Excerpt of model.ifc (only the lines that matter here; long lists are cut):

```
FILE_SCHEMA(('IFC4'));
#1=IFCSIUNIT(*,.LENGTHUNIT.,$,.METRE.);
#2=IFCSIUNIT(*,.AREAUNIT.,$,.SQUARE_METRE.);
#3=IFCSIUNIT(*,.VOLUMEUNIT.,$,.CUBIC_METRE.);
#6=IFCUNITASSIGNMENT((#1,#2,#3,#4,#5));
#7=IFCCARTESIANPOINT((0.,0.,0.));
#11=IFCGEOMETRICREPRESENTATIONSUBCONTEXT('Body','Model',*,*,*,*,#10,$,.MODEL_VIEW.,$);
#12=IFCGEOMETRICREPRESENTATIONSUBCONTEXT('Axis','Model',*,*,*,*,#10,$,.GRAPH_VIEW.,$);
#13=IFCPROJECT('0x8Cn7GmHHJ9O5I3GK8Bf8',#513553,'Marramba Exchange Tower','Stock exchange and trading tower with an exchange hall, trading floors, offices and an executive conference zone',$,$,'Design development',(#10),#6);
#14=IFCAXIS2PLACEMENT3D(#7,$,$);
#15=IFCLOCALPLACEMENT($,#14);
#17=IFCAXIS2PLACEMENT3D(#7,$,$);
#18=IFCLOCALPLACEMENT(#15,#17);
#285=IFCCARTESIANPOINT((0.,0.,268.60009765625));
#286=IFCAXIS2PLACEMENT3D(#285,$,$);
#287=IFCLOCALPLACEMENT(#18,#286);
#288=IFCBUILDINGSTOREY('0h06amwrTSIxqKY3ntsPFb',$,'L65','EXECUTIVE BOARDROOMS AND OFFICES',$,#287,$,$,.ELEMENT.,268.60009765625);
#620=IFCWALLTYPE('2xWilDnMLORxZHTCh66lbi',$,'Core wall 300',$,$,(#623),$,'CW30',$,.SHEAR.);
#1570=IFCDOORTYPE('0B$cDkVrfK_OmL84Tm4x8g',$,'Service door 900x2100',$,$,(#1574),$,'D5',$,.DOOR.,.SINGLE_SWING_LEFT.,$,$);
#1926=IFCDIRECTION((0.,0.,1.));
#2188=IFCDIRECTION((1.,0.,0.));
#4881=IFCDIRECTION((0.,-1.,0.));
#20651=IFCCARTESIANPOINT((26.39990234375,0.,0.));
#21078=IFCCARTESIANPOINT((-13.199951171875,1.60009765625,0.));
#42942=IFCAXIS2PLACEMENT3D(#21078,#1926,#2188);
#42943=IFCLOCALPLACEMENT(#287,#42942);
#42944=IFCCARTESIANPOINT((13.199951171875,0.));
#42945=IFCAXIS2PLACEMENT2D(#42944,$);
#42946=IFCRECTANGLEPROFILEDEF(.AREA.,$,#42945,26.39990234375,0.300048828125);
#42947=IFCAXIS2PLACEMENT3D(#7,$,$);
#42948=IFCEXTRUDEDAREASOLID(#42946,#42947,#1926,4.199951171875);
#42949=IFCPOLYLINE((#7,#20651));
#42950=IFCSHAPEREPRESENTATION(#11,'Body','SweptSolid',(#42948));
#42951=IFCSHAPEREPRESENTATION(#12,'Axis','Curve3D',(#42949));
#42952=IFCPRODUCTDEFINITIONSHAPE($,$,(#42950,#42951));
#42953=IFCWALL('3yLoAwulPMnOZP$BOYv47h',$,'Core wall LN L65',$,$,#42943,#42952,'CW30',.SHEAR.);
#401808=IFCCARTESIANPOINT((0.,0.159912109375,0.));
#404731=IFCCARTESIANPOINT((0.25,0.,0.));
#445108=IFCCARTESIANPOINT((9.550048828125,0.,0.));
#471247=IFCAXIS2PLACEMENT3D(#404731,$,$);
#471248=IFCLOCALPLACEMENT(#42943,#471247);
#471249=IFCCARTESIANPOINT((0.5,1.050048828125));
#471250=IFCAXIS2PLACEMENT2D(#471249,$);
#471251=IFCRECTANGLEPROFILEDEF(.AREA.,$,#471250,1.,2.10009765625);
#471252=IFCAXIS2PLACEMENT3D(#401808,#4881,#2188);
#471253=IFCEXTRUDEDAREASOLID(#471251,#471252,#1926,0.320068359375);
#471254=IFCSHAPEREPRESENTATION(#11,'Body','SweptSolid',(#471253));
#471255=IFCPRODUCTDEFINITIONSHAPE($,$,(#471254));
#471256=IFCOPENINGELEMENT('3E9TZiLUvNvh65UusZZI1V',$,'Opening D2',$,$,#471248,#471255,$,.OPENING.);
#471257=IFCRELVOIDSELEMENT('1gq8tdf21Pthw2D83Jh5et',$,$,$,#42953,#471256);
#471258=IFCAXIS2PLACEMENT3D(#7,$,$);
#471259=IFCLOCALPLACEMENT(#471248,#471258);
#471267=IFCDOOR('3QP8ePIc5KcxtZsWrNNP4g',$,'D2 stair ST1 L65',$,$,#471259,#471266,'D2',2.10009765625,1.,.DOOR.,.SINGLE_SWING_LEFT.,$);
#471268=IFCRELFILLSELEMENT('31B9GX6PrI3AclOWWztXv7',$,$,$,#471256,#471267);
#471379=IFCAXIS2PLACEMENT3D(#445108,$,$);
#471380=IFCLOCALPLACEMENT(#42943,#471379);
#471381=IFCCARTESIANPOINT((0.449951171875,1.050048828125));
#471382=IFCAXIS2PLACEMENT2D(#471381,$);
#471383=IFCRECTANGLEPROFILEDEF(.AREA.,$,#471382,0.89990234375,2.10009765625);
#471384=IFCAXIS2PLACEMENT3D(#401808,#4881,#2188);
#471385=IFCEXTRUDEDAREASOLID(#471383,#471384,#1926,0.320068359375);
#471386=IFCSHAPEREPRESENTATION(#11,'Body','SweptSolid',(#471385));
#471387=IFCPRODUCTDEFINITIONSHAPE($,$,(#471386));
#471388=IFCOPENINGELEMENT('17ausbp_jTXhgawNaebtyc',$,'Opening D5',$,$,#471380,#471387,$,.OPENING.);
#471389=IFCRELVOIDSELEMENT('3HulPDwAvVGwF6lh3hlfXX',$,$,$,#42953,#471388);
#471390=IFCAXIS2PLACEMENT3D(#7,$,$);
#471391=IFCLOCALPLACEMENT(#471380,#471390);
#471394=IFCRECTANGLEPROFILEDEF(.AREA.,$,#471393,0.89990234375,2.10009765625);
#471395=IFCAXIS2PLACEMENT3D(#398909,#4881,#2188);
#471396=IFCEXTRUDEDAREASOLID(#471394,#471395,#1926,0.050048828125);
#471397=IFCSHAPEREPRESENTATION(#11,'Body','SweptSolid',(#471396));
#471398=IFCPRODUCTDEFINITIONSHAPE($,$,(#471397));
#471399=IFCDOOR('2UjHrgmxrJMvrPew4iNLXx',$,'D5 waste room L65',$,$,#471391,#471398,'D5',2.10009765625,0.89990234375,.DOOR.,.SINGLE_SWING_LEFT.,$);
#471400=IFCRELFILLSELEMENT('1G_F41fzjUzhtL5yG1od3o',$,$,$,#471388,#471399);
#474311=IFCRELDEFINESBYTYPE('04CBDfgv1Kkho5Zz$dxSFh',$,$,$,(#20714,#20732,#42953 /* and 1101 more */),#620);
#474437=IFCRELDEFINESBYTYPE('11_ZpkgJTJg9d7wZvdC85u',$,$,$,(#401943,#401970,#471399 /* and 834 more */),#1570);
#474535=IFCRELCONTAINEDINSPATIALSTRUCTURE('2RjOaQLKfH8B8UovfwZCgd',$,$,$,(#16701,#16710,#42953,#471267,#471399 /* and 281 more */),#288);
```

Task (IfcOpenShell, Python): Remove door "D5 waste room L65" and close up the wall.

```python
import ifcopenshell
import ifcopenshell.api.feature
import ifcopenshell.api.root
import ifcopenshell.geom
import ifcopenshell.util.shape

model = ifcopenshell.open("model.ifc")
settings = ifcopenshell.geom.settings()


def volume(element):
    """Net volume in cubic metres, openings subtracted."""
    shape = ifcopenshell.geom.create_shape(settings, element)
    return ifcopenshell.util.shape.get_volume(shape.geometry)


door = model.by_id(471399)
opening = door.FillsVoids[0].RelatingOpeningElement
wall = opening.VoidsElements[0].RelatingBuildingElement
before = volume(wall)

ifcopenshell.api.root.remove_product(model, product=door)
ifcopenshell.api.feature.remove_feature(model, feature=opening)

after = volume(wall)

print(f"wall volume {before:.3f} -> {after:.3f} m3")

model.write("model_edited.ifc")
```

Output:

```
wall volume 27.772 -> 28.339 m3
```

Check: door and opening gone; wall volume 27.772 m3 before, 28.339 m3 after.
